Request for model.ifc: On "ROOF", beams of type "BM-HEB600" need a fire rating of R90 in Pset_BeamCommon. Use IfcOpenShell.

First a look at what the model holds.

```python
import ifcopenshell
import ifcopenshell.util.element

model = ifcopenshell.open("model.ifc")
print(model.schema)
storey = next(s for s in model.by_type("IfcBuildingStorey") if s.Name == "ROOF")
beams = [e for e in ifcopenshell.util.element.get_decomposition(storey) if e.is_a("IfcBeam")]
seen = {}
for e in beams:
    element_type = ifcopenshell.util.element.get_type(e)
    key = (element_type.Name if element_type != e and element_type else None, ifcopenshell.util.element.get_pset(e, "Pset_BeamCommon", "FireRating"))
    seen[key] = seen.get(key, 0) + 1
for (name, value), count in sorted(seen.items(), key=str):
    print(count, "x", name, "|", value)
```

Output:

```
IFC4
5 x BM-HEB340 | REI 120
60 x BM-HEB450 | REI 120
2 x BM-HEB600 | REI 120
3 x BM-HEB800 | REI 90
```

```python
import ifcopenshell
import ifcopenshell.api.pset
import ifcopenshell.util.element

model = ifcopenshell.open("model.ifc")

storey = next(s for s in model.by_type("IfcBuildingStorey") if s.Name == "ROOF")
beams = [e for e in ifcopenshell.util.element.get_decomposition(storey) if e.is_a("IfcBeam")]

count = 0
for e in beams:
    element_type = ifcopenshell.util.element.get_type(e)
    if element_type in (None, e) or element_type.Name != "BM-HEB600":
        continue
    # add_pset returns the element's existing set when there is one.
    pset = ifcopenshell.api.pset.add_pset(model, product=e, name="Pset_BeamCommon")
    ifcopenshell.api.pset.edit_pset(model, pset=pset, properties={"FireRating": "R90"})
    count += 1

print(count, "beams updated")

model.write("model-out.ifc")
```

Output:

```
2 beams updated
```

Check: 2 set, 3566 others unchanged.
